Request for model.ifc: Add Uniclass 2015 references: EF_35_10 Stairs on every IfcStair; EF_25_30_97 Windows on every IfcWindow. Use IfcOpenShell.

First a look at what the model holds.

```python
import ifcopenshell

model = ifcopenshell.open("model.ifc")
print(model.schema)
print("classifications:", [c.Name for c in model.by_type("IfcClassification")])
for ifc_class in ("IfcDoor", "IfcRoof", "IfcStair", "IfcWall", "IfcWindow"):
    print(ifc_class, len(model.by_type(ifc_class)))
```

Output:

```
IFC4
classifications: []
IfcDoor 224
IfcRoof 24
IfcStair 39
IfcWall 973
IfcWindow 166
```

```python
import ifcopenshell
import ifcopenshell.api.classification

model = ifcopenshell.open("model.ifc")

system = ifcopenshell.api.classification.add_classification(model, classification="Uniclass 2015")

codes = {
    "IfcStair": ("EF_35_10", "Stairs"),
    "IfcWindow": ("EF_25_30_97", "Windows"),
}
for ifc_class, (code, name) in codes.items():
    products = model.by_type(ifc_class)
    ifcopenshell.api.classification.add_reference(
        model, products=products, classification=system, identification=code, name=name
    )
    print(code, len(products))

model.write("model_rev.ifc")
```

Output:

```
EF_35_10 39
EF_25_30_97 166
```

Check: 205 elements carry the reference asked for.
